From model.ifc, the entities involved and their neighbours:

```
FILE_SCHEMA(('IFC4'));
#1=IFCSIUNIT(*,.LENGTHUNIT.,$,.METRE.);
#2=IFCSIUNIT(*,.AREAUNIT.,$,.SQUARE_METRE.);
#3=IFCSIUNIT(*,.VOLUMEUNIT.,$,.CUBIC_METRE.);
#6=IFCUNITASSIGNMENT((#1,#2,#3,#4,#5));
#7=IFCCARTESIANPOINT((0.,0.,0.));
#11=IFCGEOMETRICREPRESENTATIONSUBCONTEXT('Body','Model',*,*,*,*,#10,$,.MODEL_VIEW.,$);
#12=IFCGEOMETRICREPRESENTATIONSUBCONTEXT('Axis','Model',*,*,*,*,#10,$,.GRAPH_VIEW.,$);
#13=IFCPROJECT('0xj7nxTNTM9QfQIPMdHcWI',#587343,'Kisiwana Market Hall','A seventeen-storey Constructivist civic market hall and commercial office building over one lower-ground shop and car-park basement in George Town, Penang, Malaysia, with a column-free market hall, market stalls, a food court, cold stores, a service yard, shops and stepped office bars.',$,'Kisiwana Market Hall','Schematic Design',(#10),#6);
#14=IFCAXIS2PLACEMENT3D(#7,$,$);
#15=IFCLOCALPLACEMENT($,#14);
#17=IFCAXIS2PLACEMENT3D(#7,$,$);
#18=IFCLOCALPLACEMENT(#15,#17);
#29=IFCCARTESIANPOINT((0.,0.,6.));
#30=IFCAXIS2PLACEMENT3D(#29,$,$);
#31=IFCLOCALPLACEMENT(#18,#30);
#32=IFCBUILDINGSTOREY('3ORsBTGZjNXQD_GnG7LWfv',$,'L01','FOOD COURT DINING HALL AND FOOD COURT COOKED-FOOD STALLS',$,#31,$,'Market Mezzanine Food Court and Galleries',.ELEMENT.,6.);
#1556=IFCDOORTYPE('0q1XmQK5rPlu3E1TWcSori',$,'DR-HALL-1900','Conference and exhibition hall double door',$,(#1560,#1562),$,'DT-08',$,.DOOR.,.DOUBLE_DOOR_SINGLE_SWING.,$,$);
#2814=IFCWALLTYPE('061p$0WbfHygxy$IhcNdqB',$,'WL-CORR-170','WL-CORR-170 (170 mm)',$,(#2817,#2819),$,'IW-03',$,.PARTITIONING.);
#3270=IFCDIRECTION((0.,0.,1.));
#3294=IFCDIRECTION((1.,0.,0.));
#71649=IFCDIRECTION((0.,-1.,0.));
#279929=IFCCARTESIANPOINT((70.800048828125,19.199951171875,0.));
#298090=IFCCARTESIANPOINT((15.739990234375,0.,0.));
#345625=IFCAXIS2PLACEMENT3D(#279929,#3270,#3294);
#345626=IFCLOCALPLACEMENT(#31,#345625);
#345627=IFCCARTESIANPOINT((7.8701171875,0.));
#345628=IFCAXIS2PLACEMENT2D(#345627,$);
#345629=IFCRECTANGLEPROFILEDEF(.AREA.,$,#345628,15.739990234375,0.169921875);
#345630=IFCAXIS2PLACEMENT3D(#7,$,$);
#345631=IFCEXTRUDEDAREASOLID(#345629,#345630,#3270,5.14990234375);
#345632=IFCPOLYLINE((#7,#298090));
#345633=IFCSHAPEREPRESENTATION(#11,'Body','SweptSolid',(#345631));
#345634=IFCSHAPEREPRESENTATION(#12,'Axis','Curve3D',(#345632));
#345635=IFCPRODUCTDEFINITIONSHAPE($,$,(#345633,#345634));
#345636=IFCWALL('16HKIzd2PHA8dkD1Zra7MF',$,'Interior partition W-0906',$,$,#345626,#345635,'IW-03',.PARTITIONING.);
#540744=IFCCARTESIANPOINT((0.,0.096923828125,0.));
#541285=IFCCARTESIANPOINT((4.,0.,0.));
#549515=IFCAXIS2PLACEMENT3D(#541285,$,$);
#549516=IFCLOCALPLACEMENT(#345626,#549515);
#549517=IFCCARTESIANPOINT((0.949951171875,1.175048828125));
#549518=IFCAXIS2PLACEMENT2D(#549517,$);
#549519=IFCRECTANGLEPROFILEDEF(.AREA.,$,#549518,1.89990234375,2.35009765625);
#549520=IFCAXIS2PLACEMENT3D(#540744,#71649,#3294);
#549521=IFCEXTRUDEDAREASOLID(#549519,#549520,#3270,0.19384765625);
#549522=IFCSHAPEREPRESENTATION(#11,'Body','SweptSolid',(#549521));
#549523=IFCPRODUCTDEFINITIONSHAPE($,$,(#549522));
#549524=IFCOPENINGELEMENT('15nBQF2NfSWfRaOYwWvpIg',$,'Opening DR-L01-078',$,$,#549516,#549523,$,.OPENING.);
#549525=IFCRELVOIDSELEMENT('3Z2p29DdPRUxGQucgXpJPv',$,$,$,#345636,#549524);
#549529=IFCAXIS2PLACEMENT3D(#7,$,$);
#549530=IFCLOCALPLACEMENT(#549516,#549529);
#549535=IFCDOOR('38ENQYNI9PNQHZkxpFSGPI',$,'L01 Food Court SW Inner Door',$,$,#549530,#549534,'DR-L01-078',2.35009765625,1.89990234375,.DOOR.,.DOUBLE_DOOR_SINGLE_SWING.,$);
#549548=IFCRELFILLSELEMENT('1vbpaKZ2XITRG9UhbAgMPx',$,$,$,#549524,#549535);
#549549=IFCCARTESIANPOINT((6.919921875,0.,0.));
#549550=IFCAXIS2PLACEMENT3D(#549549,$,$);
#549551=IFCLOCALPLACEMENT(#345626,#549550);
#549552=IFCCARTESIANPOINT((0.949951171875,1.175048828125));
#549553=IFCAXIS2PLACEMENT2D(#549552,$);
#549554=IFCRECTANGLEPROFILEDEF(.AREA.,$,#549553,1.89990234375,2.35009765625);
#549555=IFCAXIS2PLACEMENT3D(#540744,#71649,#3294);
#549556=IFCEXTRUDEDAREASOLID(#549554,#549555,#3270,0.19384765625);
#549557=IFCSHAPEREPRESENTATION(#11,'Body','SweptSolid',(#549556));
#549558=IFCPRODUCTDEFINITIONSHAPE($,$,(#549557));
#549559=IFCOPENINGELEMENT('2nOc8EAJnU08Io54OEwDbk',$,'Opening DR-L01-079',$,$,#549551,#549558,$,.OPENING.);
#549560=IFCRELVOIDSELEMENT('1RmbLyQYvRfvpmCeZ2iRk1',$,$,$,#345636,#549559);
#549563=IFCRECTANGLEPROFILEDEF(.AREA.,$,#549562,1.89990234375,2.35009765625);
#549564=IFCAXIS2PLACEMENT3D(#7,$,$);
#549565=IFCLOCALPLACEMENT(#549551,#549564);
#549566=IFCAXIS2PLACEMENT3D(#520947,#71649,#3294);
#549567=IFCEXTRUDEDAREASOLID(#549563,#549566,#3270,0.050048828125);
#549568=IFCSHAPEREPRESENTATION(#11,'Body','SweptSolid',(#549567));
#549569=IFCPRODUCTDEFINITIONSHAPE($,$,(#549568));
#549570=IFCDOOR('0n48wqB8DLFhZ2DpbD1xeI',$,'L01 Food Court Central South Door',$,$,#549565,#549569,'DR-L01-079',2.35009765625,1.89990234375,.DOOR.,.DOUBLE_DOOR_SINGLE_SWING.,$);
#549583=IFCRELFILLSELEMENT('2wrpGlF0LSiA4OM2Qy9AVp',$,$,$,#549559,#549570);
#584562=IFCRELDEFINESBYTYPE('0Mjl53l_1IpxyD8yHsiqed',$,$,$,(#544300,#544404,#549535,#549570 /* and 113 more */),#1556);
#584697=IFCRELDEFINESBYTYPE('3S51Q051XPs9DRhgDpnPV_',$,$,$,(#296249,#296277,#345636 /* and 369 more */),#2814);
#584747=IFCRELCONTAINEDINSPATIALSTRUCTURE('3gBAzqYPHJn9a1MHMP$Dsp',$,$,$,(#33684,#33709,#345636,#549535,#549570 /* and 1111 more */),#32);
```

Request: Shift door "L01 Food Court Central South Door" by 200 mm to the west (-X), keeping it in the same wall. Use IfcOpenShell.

```python
import ifcopenshell
import ifcopenshell.api.geometry
import ifcopenshell.util.placement

model = ifcopenshell.open("model.ifc")

door = model.by_guid("0n48wqB8DLFhZ2DpbD1xeI")
opening = door.FillsVoids[0].RelatingOpeningElement
wall = opening.VoidsElements[0].RelatingBuildingElement

wall_matrix = ifcopenshell.util.placement.get_local_placement(wall.ObjectPlacement)
shift = wall_matrix[:3, 0] * -0.2
before = ifcopenshell.util.placement.get_local_placement(door.ObjectPlacement)[:3, 3].copy()

# The door is placed relative to its opening, so it follows when the opening moves.
matrix = ifcopenshell.util.placement.get_local_placement(opening.ObjectPlacement)
matrix[:3, 3] += shift
ifcopenshell.api.geometry.edit_object_placement(
    model, product=opening, matrix=matrix, is_si=False, should_transform_children=True
)

after = ifcopenshell.util.placement.get_local_placement(door.ObjectPlacement)[:3, 3]
print("door moved by", (after - before).round(3) + 0.0)

model.write("model_rev.ifc")
```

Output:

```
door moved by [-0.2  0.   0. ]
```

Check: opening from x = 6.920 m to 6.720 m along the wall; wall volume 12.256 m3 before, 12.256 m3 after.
